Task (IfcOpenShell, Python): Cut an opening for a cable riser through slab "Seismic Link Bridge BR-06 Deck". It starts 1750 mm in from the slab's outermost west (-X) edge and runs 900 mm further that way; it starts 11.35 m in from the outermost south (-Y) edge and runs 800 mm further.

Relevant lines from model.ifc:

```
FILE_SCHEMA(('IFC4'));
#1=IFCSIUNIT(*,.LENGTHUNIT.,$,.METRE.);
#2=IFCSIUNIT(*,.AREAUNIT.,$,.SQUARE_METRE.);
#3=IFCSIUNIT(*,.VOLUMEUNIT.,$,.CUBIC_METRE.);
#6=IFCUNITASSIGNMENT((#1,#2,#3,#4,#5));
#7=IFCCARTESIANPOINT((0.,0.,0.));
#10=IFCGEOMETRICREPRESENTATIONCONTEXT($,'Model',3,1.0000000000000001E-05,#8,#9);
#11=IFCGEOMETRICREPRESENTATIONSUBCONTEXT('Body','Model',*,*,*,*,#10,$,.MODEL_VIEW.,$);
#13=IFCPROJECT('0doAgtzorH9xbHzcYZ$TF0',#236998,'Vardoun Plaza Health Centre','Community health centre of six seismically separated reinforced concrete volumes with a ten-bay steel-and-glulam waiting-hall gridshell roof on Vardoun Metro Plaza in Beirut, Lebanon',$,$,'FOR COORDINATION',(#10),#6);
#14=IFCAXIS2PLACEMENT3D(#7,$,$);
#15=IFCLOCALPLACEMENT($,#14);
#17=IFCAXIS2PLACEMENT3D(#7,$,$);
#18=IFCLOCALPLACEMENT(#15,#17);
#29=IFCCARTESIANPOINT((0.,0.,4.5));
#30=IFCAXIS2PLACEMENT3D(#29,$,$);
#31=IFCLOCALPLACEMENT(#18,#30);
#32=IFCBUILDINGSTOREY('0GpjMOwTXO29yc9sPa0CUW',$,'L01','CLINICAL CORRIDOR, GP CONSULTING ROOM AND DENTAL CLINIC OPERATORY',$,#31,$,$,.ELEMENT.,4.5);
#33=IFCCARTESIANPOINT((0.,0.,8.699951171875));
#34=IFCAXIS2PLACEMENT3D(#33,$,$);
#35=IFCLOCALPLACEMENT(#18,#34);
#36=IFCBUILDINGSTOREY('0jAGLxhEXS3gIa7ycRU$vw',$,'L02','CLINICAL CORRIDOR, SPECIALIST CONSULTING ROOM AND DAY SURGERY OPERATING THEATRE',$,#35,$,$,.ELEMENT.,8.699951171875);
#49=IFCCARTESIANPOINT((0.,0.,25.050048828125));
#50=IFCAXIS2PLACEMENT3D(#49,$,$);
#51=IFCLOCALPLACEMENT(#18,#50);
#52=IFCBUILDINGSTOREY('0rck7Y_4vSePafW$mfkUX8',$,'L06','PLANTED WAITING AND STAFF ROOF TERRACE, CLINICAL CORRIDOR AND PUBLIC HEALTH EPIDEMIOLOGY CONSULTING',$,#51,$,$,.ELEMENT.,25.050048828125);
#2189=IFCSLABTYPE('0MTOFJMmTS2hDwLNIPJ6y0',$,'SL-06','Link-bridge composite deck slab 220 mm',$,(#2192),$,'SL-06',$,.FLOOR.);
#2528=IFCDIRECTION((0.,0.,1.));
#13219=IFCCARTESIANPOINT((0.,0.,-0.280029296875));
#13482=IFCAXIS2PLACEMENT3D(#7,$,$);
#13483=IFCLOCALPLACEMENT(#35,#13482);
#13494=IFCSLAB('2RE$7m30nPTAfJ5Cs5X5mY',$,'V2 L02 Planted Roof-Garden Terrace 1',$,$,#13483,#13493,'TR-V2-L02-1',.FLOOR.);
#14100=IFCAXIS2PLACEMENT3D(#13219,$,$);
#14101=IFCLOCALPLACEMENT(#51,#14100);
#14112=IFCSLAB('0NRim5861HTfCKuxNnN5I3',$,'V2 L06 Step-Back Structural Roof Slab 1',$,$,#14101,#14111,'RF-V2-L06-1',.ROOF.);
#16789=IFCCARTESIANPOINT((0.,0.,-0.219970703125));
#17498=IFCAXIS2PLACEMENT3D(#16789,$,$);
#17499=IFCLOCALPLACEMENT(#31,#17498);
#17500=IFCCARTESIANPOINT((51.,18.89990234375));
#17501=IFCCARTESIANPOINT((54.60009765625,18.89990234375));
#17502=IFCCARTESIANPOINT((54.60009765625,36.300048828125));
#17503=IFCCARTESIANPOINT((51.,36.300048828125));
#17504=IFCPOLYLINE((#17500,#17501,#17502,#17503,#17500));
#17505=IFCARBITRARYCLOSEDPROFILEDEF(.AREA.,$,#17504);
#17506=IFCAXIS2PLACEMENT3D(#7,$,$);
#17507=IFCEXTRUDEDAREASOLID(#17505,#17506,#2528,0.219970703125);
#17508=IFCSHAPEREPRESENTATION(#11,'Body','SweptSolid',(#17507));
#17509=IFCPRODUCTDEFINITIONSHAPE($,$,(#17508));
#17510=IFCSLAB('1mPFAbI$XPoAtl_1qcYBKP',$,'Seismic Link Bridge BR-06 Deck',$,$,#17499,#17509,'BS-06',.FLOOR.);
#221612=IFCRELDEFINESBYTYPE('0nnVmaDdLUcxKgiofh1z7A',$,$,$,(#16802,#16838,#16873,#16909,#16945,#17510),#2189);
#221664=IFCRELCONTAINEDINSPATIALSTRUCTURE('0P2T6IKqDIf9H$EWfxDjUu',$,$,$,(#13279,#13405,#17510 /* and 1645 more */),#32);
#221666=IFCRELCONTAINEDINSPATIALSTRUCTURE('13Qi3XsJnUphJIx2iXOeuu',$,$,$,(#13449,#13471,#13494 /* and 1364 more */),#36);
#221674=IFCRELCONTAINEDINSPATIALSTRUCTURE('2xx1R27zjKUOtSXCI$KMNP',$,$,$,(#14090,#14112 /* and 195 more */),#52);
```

```python
import numpy as np
import ifcopenshell
import ifcopenshell.api.feature
import ifcopenshell.api.geometry
import ifcopenshell.api.root
import ifcopenshell.geom
import ifcopenshell.util.placement
import ifcopenshell.util.representation
import ifcopenshell.util.shape
import ifcopenshell.util.unit

model = ifcopenshell.open("model.ifc")
unit_scale = ifcopenshell.util.unit.calculate_unit_scale(model)
settings = ifcopenshell.geom.settings()


def volume(element):
    """Net volume in cubic metres, openings subtracted."""
    shape = ifcopenshell.geom.create_shape(settings, element)
    return ifcopenshell.util.shape.get_volume(shape.geometry)


slab = model.by_guid("1mPFAbI$XPoAtl_1qcYBKP")
before = volume(slab)

# Extent in the slab's own axes, in metres. The edges named are its -X and -Y sides.
slab_shape = ifcopenshell.geom.create_shape(settings, slab)
vertices = ifcopenshell.util.shape.get_vertices(slab_shape.geometry)
x_min, y_min, bottom = vertices.min(axis=0)
top = vertices[:, 2].max()

opening = ifcopenshell.api.root.create_entity(model, ifc_class="IfcOpeningElement", name="Cable riser opening", predefined_type="OPENING")
context = ifcopenshell.util.representation.get_context(model, "Model", "Body", "MODEL_VIEW")
width, depth = 0.9, 0.8
outline = [(0.0, 0.0), (width, 0.0), (width, depth), (0.0, depth), (0.0, 0.0)]
# Overshoot both faces by 50 mm so the cut is clean.
shape = ifcopenshell.api.geometry.add_slab_representation(
    model, context=context, depth=top - bottom + 0.1, polyline=outline
)
ifcopenshell.api.geometry.assign_representation(model, product=opening, representation=shape)

matrix = ifcopenshell.util.placement.get_local_placement(slab.ObjectPlacement)
matrix[:, 3] = matrix @ np.append(np.array([x_min + 1.75, y_min + 11.35, bottom - 0.05]) / unit_scale, 1.0)
ifcopenshell.api.geometry.edit_object_placement(model, product=opening, matrix=matrix, is_si=False)
ifcopenshell.api.feature.add_feature(model, feature=opening, element=slab)

after = volume(slab)

print(f"slab volume {before:.3f} -> {after:.3f} m3")

model.write("model_rev.ifc")
```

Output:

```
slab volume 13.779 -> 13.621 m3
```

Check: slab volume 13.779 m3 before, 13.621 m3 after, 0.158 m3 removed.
